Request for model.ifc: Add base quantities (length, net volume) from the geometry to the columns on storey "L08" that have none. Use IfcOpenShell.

First a look at what the model holds.

```python
import ifcopenshell
import ifcopenshell.util.element
import ifcopenshell.util.unit

model = ifcopenshell.open("model.ifc")
print(model.schema)
for unit_type in ("LENGTHUNIT", "AREAUNIT", "VOLUMEUNIT"):
    print(unit_type, ifcopenshell.util.unit.calculate_unit_scale(model, unit_type))
storey = next(s for s in model.by_type("IfcBuildingStorey") if s.Name == "L08")
columns = [e for e in ifcopenshell.util.element.get_decomposition(storey) if e.is_a("IfcColumn")]
for e in sorted(columns, key=lambda e: e.id()):
    print(e.id(), e.is_a(), e.Name, list(ifcopenshell.util.element.get_psets(e, qtos_only=True)), sep=" | ")
```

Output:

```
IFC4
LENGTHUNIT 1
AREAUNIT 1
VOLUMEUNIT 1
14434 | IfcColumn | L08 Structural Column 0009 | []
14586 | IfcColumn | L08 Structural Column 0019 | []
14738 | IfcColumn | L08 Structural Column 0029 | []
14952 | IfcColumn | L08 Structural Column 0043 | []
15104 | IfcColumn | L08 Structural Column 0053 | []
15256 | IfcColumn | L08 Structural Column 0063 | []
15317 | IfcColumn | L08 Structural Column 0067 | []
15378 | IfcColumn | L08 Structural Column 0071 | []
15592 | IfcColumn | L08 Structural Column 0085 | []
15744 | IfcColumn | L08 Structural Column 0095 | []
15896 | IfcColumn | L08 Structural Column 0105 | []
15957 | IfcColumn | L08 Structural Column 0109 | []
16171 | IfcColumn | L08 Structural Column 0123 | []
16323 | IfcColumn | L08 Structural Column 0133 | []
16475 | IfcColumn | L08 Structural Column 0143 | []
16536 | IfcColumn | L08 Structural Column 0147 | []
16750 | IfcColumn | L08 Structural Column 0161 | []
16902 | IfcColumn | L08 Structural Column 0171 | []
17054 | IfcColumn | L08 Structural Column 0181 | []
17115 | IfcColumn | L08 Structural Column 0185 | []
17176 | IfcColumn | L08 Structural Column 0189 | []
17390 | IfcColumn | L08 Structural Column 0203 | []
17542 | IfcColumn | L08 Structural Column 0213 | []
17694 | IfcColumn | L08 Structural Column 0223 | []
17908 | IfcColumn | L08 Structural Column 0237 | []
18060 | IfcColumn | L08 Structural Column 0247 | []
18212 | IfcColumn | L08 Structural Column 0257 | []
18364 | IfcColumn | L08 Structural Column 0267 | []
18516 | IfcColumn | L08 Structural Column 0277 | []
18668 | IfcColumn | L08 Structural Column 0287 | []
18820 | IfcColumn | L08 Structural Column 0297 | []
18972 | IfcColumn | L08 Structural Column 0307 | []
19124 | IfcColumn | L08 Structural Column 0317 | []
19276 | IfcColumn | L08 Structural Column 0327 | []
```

```python
import ifcopenshell
import ifcopenshell.api.pset
import ifcopenshell.geom
import ifcopenshell.util.element
import ifcopenshell.util.shape
import ifcopenshell.util.unit

model = ifcopenshell.open("model.ifc")
unit_scale = ifcopenshell.util.unit.calculate_unit_scale(model)
volume_scale = ifcopenshell.util.unit.calculate_unit_scale(model, "VOLUMEUNIT")
settings = ifcopenshell.geom.settings()

storey = next(s for s in model.by_type("IfcBuildingStorey") if s.Name == "L08")
columns = [e for e in ifcopenshell.util.element.get_decomposition(storey) if e.is_a("IfcColumn")]

for e in sorted(columns, key=lambda e: e.id()):
    if ifcopenshell.util.element.get_psets(e, qtos_only=True, should_inherit=False):
        continue
    # Geometry comes back in metres, in the element's own axes.
    shape = ifcopenshell.geom.create_shape(settings, e)
    values = {
        "Length": ifcopenshell.util.shape.get_z(shape.geometry) / unit_scale,
        "NetVolume": ifcopenshell.util.shape.get_volume(shape.geometry) / volume_scale,
    }
    qto = ifcopenshell.api.pset.add_qto(model, product=e, name="Qto_ColumnBaseQuantities")
    ifcopenshell.api.pset.edit_qto(model, qto=qto, properties=values)
    print(e.id(), {k: round(v, 3) for k, v in values.items()})

model.write("model_updated.ifc")
```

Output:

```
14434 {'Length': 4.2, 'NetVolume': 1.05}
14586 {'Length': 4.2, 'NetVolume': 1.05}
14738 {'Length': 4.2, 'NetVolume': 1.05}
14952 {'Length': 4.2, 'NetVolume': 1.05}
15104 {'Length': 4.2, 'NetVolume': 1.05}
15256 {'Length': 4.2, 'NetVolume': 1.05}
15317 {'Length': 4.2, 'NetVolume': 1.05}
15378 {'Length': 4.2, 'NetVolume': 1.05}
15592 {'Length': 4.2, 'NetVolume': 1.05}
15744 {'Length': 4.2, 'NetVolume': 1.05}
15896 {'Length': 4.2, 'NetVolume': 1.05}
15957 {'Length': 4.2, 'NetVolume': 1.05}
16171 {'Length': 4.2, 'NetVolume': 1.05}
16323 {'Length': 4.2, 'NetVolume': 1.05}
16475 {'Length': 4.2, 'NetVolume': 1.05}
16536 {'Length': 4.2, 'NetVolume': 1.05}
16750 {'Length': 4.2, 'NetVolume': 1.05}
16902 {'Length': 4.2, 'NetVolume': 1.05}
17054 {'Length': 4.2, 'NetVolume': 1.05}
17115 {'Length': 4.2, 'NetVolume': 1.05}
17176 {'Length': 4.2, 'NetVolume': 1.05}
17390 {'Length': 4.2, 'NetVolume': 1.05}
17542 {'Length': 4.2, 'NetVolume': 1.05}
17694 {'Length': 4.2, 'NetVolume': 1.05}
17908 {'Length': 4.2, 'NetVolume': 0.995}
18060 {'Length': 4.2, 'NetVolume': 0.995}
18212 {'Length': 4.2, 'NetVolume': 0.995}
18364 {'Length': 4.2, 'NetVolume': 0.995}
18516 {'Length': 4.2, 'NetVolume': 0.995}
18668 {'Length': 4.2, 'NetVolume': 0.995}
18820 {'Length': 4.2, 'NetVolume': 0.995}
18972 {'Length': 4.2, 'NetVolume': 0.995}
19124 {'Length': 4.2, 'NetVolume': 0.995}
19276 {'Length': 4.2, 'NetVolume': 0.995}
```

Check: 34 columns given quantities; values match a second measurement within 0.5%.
